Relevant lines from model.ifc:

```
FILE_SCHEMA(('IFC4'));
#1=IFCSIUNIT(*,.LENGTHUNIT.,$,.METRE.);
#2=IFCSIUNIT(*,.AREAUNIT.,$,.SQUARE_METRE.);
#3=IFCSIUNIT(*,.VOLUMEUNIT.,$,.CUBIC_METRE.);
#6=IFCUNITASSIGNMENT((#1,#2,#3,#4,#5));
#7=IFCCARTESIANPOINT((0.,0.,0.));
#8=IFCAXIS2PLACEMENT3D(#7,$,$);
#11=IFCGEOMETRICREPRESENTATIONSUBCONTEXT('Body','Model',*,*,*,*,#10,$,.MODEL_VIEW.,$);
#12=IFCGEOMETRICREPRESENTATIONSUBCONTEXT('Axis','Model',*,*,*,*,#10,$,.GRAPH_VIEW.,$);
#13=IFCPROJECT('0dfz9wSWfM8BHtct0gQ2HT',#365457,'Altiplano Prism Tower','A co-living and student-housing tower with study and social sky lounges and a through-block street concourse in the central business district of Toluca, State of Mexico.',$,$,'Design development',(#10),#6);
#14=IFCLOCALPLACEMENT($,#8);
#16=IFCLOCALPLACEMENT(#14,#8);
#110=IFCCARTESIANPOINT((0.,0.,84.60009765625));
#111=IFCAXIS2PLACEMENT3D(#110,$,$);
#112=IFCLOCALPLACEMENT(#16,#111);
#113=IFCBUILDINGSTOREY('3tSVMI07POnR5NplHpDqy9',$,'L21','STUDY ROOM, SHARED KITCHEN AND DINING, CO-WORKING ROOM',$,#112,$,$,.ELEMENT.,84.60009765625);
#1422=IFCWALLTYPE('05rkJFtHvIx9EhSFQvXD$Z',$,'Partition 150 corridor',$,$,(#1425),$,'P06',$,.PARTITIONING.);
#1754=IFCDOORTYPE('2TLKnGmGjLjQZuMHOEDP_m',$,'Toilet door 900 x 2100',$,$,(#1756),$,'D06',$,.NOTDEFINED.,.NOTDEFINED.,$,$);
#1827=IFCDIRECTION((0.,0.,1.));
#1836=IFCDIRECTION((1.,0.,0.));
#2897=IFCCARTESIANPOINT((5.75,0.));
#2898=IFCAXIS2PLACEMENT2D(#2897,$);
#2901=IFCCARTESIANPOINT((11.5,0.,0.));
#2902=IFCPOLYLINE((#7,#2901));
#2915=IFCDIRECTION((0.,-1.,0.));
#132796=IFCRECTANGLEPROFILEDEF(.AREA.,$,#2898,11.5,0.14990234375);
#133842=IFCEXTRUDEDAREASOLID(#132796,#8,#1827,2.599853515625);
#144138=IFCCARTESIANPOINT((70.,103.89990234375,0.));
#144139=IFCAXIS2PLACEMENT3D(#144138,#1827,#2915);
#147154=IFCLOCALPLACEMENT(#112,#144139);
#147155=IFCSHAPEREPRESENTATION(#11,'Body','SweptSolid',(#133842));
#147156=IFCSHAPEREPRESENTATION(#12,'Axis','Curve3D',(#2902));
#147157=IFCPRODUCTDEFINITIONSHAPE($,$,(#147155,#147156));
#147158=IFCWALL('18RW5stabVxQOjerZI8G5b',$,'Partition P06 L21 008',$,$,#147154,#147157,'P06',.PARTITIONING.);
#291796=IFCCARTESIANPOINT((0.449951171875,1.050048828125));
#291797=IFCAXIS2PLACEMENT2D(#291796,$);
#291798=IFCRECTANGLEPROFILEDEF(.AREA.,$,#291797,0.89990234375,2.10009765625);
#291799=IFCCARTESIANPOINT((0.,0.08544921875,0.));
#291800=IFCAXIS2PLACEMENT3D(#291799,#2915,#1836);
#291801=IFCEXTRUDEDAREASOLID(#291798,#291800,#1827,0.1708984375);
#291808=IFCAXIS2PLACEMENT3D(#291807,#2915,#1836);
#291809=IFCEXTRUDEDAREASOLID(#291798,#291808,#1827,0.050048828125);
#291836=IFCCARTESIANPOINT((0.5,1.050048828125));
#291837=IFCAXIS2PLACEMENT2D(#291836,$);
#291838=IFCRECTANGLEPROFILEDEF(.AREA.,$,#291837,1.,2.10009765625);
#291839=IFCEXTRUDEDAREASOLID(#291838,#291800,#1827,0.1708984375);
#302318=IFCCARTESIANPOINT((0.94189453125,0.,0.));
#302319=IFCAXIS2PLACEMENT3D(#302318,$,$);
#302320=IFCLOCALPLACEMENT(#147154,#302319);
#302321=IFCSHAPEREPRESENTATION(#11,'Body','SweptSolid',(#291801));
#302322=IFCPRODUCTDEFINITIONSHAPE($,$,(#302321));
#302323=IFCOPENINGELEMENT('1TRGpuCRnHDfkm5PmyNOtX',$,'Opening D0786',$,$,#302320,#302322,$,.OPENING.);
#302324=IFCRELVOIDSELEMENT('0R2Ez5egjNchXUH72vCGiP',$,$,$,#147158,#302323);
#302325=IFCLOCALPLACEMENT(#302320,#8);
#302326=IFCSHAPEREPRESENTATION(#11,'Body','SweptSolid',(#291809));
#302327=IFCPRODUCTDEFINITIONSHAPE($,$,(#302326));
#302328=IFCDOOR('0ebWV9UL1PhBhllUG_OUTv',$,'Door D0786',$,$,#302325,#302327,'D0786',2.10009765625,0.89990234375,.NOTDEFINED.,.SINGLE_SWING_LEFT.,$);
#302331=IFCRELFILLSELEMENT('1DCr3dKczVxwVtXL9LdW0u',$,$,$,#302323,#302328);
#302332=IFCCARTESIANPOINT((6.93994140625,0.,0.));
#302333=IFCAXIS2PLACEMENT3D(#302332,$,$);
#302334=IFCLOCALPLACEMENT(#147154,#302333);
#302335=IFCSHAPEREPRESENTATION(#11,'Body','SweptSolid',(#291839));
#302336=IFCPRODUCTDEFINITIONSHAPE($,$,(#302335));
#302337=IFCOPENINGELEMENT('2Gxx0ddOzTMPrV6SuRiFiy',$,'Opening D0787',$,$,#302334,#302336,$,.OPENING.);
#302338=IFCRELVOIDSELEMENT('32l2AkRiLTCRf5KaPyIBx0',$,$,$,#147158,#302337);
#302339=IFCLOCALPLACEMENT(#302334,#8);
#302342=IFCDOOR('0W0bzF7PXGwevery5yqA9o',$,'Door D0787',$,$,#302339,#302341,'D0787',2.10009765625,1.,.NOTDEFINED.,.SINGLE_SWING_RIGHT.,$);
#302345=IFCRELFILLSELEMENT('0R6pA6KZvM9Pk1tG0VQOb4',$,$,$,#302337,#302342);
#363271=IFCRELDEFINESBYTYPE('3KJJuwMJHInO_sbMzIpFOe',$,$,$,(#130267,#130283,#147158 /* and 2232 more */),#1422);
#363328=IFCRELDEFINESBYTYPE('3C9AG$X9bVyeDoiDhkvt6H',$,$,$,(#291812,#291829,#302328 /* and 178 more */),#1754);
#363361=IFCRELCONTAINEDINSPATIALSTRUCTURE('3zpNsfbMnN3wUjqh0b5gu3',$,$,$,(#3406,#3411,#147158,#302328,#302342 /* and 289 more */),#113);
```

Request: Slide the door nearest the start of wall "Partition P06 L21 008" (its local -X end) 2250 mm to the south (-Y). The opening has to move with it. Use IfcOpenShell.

```python
import ifcopenshell
import ifcopenshell.api.geometry
import ifcopenshell.util.placement
import ifcopenshell.util.unit

model = ifcopenshell.open("model.ifc")
unit_scale = ifcopenshell.util.unit.calculate_unit_scale(model)

door = model.by_guid("0ebWV9UL1PhBhllUG_OUTv")
opening = door.FillsVoids[0].RelatingOpeningElement
wall = opening.VoidsElements[0].RelatingBuildingElement

wall_matrix = ifcopenshell.util.placement.get_local_placement(wall.ObjectPlacement)
shift = wall_matrix[:3, 0] * 2.25 / unit_scale
before = ifcopenshell.util.placement.get_local_placement(door.ObjectPlacement)[:3, 3].copy()

# The door is placed relative to its opening, so it follows when the opening moves.
matrix = ifcopenshell.util.placement.get_local_placement(opening.ObjectPlacement)
matrix[:3, 3] += shift
ifcopenshell.api.geometry.edit_object_placement(
    model, product=opening, matrix=matrix, is_si=False, should_transform_children=True
)

after = ifcopenshell.util.placement.get_local_placement(door.ObjectPlacement)[:3, 3]
print("door moved by", (after - before).round(3) + 0.0)

model.write("model_v2.ifc")
```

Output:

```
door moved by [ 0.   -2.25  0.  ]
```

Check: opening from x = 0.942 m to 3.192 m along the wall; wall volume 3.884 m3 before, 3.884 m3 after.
